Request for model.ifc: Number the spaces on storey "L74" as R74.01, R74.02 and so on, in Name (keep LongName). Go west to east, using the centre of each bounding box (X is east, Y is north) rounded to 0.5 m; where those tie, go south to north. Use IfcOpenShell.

First a look at what the model holds.

```python
import ifcopenshell
import ifcopenshell.util.element
import ifcopenshell.util.placement

model = ifcopenshell.open("model.ifc")
print(model.schema)
storey = next(s for s in model.by_type("IfcBuildingStorey") if s.Name == "L74")
spaces = [e for e in ifcopenshell.util.element.get_decomposition(storey) if e.is_a("IfcSpace")]
for e in sorted(spaces, key=lambda e: e.id()):
    origin = ifcopenshell.util.placement.get_local_placement(e.ObjectPlacement)[:3, 3]
    print(e.id(), e.Name, e.LongName, origin.round(2) + 0.0, sep=" | ")
```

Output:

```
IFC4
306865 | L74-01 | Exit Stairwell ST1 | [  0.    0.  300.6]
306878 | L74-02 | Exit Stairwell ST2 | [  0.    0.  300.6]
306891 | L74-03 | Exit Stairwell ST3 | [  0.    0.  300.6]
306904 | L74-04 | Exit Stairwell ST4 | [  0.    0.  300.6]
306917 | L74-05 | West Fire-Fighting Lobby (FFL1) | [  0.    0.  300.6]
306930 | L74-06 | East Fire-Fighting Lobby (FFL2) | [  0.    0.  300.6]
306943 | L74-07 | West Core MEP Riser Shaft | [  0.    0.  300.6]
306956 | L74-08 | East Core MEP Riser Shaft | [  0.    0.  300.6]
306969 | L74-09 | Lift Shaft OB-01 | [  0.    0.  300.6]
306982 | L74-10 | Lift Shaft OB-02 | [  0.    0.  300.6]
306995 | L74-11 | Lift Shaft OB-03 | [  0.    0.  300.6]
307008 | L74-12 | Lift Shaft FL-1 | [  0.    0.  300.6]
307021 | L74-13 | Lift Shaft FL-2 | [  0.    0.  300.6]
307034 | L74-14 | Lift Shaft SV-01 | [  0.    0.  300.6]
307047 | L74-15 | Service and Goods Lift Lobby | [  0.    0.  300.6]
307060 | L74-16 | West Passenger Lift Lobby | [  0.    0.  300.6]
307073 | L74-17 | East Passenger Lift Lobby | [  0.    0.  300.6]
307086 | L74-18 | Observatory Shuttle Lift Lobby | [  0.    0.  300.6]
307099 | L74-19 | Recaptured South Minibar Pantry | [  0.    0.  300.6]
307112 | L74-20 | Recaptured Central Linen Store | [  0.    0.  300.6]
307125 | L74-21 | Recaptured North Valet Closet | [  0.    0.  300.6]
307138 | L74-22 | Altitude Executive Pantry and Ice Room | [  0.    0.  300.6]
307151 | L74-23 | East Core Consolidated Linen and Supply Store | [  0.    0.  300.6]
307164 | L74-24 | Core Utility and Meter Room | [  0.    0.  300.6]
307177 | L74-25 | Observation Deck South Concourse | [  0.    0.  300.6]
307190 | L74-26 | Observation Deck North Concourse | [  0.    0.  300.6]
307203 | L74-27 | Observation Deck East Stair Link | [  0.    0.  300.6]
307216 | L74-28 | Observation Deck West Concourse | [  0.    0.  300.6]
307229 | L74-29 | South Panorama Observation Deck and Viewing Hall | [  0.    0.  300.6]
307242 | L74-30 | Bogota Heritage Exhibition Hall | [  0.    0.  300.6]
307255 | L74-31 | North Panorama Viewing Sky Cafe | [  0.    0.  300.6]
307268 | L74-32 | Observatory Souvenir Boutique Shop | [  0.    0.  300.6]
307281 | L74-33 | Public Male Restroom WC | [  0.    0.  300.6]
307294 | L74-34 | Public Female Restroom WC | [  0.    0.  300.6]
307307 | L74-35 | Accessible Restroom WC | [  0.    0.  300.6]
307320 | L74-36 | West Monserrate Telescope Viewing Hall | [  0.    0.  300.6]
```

```python
import ifcopenshell
import ifcopenshell.geom
import ifcopenshell.util.element
import ifcopenshell.util.shape

model = ifcopenshell.open("model.ifc")
settings = ifcopenshell.geom.settings()
settings.set("use-world-coords", True)


def centre(element):
    shape = ifcopenshell.geom.create_shape(settings, element)
    return ifcopenshell.util.shape.get_bbox_centroid(shape.geometry)


storey = next(s for s in model.by_type("IfcBuildingStorey") if s.Name == "L74")
spaces = [e for e in ifcopenshell.util.element.get_decomposition(storey) if e.is_a("IfcSpace")]

# Insertion points can sit at a corner or the storey origin, so sort by the geometry (in metres).
centres = {e: centre(e) for e in spaces}
spaces.sort(key=lambda e: (round(centres[e][0] / 0.5), centres[e][1]))

for i, e in enumerate(spaces, start=1):
    number = f"R74.{i:02d}"
    e.Name = number
    print(e.id(), number)

model.write("model_v2.ifc")
```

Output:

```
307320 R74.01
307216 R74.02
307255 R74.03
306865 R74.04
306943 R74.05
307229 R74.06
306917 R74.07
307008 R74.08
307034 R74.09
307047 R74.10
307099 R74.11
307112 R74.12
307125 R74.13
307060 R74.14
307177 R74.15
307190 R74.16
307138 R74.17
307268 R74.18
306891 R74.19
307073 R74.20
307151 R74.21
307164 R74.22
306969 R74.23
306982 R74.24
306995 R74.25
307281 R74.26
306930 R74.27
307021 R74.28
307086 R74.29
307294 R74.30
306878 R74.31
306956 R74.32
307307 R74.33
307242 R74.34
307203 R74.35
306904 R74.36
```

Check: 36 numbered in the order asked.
